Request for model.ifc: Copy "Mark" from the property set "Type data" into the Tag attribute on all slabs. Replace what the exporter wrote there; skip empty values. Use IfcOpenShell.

First a look at what the model holds.

```python
import ifcopenshell
import ifcopenshell.util.element

model = ifcopenshell.open("model.ifc")
print(model.schema)
slabs = model.by_type("IfcSlab")
print(len(slabs), "slabs")
for e in slabs[:8]:
    source = ifcopenshell.util.element.get_pset(e, "Type data", "Mark")
    target = e.Tag
    print(e.id(), repr(source), repr(target), sep=" | ")
```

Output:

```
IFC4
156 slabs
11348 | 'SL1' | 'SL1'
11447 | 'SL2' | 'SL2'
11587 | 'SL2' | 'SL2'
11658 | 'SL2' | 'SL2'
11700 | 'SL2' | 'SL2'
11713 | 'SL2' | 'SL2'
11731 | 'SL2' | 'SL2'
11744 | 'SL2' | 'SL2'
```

```python
import ifcopenshell
import ifcopenshell.util.element

model = ifcopenshell.open("model.ifc")

count = 0
for e in model.by_type("IfcSlab"):
    value = ifcopenshell.util.element.get_pset(e, "Type data", "Mark")
    current = e.Tag
    if not value or not value.strip() or current == value:
        continue
    e.Tag = value
    count += 1

print(count, "slabs updated")

model.write("model_updated.ifc")
```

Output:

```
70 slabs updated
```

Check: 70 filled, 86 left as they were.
